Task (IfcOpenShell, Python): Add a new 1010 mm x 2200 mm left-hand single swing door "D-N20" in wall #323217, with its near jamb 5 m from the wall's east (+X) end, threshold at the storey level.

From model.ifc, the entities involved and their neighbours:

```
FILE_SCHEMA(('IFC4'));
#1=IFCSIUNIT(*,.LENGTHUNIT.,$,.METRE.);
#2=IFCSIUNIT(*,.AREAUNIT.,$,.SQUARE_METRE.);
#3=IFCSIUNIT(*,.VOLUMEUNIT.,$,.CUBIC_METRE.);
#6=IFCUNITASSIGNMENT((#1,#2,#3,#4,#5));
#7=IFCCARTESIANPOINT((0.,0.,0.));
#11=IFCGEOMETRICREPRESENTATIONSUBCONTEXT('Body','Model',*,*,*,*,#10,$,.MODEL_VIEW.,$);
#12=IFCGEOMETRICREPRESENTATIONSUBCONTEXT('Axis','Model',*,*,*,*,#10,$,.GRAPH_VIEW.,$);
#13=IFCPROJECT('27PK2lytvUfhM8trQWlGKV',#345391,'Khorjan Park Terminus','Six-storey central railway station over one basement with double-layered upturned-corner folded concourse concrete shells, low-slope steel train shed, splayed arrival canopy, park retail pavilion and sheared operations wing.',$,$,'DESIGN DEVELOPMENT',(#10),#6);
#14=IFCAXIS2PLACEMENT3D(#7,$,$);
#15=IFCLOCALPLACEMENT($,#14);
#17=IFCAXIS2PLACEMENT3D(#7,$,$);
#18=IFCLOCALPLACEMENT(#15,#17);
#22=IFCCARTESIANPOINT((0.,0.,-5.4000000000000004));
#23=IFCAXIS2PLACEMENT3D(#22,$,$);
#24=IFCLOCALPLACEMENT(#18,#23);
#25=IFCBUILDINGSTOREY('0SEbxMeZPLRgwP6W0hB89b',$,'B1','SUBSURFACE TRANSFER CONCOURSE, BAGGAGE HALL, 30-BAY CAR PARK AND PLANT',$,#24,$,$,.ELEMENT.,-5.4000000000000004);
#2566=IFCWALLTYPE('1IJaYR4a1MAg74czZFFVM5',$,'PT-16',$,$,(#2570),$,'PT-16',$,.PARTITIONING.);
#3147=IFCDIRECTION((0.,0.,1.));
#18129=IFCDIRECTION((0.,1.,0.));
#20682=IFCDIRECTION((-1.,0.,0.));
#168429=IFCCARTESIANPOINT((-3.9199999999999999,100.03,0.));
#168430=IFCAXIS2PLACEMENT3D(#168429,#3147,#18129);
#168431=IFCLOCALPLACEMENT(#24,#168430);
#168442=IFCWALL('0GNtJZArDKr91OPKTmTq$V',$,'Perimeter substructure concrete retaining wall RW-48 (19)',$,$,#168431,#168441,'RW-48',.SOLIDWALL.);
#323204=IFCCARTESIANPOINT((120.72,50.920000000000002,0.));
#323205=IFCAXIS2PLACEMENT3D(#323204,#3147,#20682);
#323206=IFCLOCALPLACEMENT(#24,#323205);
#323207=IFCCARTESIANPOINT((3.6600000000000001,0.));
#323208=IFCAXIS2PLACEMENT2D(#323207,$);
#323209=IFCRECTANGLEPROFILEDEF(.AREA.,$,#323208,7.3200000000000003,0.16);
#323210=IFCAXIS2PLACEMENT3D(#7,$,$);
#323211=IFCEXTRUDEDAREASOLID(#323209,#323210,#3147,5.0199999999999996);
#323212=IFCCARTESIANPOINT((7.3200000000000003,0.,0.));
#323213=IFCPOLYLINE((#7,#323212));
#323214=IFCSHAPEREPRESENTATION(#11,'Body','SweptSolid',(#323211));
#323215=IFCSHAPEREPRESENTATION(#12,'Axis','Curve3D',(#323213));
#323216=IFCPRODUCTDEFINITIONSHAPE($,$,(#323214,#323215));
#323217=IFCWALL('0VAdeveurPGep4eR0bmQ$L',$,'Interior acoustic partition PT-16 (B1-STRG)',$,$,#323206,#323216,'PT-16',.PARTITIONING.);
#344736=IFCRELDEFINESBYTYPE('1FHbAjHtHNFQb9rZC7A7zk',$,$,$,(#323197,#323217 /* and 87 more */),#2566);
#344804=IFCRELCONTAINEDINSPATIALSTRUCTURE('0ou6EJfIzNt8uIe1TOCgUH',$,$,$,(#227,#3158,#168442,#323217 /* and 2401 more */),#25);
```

```python
import numpy as np
import ifcopenshell
import ifcopenshell.api.feature
import ifcopenshell.api.geometry
import ifcopenshell.api.root
import ifcopenshell.api.spatial
import ifcopenshell.geom
import ifcopenshell.util.element
import ifcopenshell.util.placement
import ifcopenshell.util.representation
import ifcopenshell.util.shape
import ifcopenshell.util.unit

model = ifcopenshell.open("model.ifc")
unit_scale = ifcopenshell.util.unit.calculate_unit_scale(model)
settings = ifcopenshell.geom.settings()


def volume(element):
    """Net volume in cubic metres, openings subtracted."""
    shape = ifcopenshell.geom.create_shape(settings, element)
    return ifcopenshell.util.shape.get_volume(shape.geometry)


wall = model.by_guid("0VAdeveurPGep4eR0bmQ$L")
storey = ifcopenshell.util.element.get_container(wall, ifc_class="IfcBuildingStorey")
context = ifcopenshell.util.representation.get_context(model, "Model", "Body", "MODEL_VIEW")
before = volume(wall)

width, height, from_end, sill = 1.01, 2.2, 5, 0.0  # metres

# The wall runs along its own X axis, and the end named is its -X end.
wall_shape = ifcopenshell.geom.create_shape(settings, wall)
x, y, z = ifcopenshell.util.shape.get_vertices(wall_shape.geometry).T
start = x.min() + from_end
face, thickness = float(y.min()), float(y.max() - y.min())
wall_matrix = ifcopenshell.util.placement.get_local_placement(wall.ObjectPlacement)
level = ifcopenshell.util.placement.get_local_placement(storey.ObjectPlacement)[2, 3]


def in_wall(x, y):
    """Placement at x, y metres in the wall's axes, at sill height."""
    matrix = wall_matrix.copy()
    matrix[:, 3] = wall_matrix @ np.array([x / unit_scale, y / unit_scale, 0.0, 1.0])
    matrix[2, 3] = level + sill / unit_scale
    return matrix


# Opening: a box that overshoots both wall faces by 50 mm.
opening = ifcopenshell.api.root.create_entity(model, ifc_class="IfcOpeningElement", predefined_type="OPENING")
box = ifcopenshell.api.geometry.add_wall_representation(
    model, context=context, length=width, height=height, thickness=thickness + 0.1
)
ifcopenshell.api.geometry.assign_representation(model, product=opening, representation=box)
ifcopenshell.api.geometry.edit_object_placement(model, product=opening, matrix=in_wall(start, face - 0.05), is_si=False)
ifcopenshell.api.feature.add_feature(model, feature=opening, element=wall)

door = ifcopenshell.api.root.create_entity(model, ifc_class="IfcDoor", name="D-N20", predefined_type="DOOR")
door.OverallWidth, door.OverallHeight = width / unit_scale, height / unit_scale
door.OperationType = "SINGLE_SWING_LEFT"
body = ifcopenshell.api.geometry.add_door_representation(
    model,
    context=context,
    overall_width=door.OverallWidth,
    overall_height=door.OverallHeight,
    operation_type="SINGLE_SWING_LEFT",
    lining_properties={"LiningDepth": thickness / unit_scale, "ThresholdDepth": thickness / unit_scale},
)
ifcopenshell.api.geometry.assign_representation(model, product=door, representation=body)
ifcopenshell.api.spatial.assign_container(model, products=[door], relating_structure=storey)
ifcopenshell.api.feature.add_filling(model, opening=opening, element=door)

# The lining spans the wall, so the door starts at the wall face.
ifcopenshell.api.geometry.edit_object_placement(model, product=door, matrix=in_wall(start, face), is_si=False)

after = volume(wall)

print(f"wall volume {before:.3f} -> {after:.3f} m3")

model.write("model_edited.ifc")
```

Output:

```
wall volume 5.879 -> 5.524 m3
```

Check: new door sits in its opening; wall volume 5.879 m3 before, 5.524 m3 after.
